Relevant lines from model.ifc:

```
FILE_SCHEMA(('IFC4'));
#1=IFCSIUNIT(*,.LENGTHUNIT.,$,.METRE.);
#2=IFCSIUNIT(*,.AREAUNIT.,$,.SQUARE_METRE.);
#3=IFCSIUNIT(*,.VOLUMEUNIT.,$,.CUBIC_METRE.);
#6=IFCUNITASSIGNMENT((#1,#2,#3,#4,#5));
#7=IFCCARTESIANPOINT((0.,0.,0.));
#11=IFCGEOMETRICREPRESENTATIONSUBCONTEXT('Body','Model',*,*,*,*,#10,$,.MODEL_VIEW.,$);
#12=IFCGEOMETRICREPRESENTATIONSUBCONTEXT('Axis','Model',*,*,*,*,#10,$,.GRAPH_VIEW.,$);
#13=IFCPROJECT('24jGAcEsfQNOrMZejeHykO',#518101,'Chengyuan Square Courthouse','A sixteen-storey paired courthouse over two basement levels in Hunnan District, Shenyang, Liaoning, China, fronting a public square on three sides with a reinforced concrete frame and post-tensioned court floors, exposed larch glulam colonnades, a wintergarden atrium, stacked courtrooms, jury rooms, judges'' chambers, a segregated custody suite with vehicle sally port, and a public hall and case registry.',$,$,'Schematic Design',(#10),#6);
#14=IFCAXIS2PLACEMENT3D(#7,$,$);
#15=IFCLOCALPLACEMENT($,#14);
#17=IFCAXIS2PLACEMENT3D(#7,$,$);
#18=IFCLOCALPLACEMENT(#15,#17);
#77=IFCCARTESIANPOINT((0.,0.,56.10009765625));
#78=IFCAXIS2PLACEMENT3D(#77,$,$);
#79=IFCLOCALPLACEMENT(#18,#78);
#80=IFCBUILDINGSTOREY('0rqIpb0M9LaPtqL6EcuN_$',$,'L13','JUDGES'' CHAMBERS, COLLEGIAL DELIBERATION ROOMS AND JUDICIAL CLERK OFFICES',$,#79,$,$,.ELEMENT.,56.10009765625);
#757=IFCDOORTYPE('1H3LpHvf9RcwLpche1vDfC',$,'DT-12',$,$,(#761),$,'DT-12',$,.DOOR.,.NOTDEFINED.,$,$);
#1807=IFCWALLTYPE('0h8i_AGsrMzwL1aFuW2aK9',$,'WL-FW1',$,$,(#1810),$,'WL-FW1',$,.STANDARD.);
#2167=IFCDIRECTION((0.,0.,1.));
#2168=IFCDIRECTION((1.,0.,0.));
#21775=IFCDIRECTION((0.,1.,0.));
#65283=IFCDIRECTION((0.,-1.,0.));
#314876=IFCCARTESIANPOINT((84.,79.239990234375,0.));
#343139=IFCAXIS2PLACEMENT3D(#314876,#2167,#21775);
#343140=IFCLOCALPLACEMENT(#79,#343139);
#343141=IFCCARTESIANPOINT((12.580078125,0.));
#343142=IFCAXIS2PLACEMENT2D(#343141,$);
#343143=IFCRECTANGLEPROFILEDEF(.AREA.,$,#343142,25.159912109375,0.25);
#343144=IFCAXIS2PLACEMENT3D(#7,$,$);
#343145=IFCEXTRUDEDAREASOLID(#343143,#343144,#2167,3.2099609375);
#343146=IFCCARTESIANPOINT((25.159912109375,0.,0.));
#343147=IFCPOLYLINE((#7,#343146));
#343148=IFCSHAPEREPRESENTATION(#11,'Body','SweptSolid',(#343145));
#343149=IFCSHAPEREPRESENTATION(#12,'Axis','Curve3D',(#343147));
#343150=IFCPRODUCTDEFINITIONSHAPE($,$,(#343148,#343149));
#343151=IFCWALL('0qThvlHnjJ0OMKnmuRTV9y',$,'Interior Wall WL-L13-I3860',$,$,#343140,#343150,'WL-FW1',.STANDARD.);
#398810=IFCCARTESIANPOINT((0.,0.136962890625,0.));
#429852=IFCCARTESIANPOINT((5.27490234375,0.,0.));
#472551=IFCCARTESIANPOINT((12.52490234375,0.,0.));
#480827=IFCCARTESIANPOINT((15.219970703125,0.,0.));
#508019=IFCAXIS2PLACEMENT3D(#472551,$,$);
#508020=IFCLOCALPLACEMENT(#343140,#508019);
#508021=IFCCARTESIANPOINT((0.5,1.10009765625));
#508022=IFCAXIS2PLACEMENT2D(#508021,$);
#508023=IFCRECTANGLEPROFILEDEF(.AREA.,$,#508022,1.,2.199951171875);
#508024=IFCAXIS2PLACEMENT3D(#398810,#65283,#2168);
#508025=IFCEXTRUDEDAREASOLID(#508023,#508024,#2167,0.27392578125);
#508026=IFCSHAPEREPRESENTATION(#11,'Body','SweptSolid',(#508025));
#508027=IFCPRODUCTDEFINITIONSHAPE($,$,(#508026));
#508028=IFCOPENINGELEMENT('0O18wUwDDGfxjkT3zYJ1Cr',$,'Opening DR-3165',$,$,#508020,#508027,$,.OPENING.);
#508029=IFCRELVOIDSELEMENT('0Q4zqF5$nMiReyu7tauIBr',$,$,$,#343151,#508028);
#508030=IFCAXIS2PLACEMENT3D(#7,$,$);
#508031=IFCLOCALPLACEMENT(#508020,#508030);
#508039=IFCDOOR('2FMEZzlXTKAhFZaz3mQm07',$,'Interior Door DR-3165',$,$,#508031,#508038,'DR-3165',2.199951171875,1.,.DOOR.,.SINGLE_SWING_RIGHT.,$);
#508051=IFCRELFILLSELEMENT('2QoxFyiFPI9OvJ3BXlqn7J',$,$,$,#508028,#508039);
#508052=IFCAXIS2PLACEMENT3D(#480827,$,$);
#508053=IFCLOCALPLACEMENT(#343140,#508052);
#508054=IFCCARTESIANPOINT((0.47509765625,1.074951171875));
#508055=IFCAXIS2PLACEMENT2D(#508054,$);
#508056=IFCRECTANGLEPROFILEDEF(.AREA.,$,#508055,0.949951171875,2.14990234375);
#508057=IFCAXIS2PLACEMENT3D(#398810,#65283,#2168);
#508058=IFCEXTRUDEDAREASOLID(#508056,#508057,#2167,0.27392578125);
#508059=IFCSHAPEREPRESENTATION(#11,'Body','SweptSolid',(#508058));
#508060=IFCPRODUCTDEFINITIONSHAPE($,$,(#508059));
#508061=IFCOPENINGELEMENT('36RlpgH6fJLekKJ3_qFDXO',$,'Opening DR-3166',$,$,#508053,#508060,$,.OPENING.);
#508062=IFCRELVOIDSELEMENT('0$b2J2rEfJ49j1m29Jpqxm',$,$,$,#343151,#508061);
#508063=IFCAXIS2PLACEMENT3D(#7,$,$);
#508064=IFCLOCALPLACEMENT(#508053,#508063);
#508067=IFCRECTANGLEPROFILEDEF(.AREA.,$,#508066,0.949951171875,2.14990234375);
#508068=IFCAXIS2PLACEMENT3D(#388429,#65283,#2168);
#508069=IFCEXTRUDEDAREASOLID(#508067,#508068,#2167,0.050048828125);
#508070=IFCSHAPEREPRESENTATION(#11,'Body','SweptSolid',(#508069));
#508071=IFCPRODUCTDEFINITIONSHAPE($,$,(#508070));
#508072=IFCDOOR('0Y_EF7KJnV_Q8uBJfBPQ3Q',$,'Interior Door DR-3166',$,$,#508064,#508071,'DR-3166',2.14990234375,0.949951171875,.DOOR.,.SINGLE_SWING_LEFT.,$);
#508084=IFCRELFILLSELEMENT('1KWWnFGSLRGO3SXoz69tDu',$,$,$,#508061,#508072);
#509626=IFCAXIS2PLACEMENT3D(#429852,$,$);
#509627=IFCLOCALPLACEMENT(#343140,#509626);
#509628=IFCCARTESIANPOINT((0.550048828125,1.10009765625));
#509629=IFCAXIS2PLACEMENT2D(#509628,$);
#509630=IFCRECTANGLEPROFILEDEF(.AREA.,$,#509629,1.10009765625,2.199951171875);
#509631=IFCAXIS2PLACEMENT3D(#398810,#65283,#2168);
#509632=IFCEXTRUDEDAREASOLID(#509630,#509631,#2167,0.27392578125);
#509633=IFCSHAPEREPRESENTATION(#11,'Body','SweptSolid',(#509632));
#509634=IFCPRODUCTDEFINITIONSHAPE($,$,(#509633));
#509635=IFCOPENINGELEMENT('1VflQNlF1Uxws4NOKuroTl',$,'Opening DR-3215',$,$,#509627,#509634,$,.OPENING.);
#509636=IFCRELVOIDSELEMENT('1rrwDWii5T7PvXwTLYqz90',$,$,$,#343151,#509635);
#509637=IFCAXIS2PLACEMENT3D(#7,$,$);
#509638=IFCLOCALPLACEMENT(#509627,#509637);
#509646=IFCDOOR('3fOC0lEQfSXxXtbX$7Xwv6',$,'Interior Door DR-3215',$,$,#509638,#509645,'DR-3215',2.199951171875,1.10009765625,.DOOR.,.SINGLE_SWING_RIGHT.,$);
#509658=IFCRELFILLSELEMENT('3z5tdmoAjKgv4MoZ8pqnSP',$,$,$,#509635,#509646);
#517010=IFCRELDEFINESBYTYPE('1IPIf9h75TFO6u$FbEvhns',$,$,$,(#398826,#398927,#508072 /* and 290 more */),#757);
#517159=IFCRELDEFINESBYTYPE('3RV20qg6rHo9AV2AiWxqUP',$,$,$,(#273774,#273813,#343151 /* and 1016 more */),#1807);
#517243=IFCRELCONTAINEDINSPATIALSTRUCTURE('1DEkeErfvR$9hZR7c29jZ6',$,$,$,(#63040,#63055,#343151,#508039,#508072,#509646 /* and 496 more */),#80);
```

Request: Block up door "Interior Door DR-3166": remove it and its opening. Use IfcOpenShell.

```python
import ifcopenshell
import ifcopenshell.api.feature
import ifcopenshell.api.root
import ifcopenshell.geom
import ifcopenshell.util.shape

model = ifcopenshell.open("model.ifc")
settings = ifcopenshell.geom.settings()


def volume(element):
    """Net volume in cubic metres, openings subtracted."""
    shape = ifcopenshell.geom.create_shape(settings, element)
    return ifcopenshell.util.shape.get_volume(shape.geometry)


door = model.by_id(508072)
opening = door.FillsVoids[0].RelatingOpeningElement
wall = opening.VoidsElements[0].RelatingBuildingElement
before = volume(wall)

ifcopenshell.api.root.remove_product(model, product=door)
ifcopenshell.api.feature.remove_feature(model, feature=opening)

after = volume(wall)

print(f"wall volume {before:.3f} -> {after:.3f} m3")

model.write("model_v2.ifc")
```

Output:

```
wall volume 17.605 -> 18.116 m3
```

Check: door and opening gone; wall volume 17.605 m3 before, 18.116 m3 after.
